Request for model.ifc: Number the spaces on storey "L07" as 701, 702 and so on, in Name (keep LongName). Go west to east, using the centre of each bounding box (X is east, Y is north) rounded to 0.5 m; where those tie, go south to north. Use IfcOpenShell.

First a look at what the model holds.

```python
import ifcopenshell
import ifcopenshell.util.element
import ifcopenshell.util.placement

model = ifcopenshell.open("model.ifc")
print(model.schema)
storey = next(s for s in model.by_type("IfcBuildingStorey") if s.Name == "L07")
spaces = [e for e in ifcopenshell.util.element.get_decomposition(storey) if e.is_a("IfcSpace")]
for e in sorted(spaces, key=lambda e: e.id()):
    origin = ifcopenshell.util.placement.get_local_placement(e.ObjectPlacement)[:3, 3]
    print(e.id(), e.Name, e.LongName, origin.round(2) + 0.0, sep=" | ")
```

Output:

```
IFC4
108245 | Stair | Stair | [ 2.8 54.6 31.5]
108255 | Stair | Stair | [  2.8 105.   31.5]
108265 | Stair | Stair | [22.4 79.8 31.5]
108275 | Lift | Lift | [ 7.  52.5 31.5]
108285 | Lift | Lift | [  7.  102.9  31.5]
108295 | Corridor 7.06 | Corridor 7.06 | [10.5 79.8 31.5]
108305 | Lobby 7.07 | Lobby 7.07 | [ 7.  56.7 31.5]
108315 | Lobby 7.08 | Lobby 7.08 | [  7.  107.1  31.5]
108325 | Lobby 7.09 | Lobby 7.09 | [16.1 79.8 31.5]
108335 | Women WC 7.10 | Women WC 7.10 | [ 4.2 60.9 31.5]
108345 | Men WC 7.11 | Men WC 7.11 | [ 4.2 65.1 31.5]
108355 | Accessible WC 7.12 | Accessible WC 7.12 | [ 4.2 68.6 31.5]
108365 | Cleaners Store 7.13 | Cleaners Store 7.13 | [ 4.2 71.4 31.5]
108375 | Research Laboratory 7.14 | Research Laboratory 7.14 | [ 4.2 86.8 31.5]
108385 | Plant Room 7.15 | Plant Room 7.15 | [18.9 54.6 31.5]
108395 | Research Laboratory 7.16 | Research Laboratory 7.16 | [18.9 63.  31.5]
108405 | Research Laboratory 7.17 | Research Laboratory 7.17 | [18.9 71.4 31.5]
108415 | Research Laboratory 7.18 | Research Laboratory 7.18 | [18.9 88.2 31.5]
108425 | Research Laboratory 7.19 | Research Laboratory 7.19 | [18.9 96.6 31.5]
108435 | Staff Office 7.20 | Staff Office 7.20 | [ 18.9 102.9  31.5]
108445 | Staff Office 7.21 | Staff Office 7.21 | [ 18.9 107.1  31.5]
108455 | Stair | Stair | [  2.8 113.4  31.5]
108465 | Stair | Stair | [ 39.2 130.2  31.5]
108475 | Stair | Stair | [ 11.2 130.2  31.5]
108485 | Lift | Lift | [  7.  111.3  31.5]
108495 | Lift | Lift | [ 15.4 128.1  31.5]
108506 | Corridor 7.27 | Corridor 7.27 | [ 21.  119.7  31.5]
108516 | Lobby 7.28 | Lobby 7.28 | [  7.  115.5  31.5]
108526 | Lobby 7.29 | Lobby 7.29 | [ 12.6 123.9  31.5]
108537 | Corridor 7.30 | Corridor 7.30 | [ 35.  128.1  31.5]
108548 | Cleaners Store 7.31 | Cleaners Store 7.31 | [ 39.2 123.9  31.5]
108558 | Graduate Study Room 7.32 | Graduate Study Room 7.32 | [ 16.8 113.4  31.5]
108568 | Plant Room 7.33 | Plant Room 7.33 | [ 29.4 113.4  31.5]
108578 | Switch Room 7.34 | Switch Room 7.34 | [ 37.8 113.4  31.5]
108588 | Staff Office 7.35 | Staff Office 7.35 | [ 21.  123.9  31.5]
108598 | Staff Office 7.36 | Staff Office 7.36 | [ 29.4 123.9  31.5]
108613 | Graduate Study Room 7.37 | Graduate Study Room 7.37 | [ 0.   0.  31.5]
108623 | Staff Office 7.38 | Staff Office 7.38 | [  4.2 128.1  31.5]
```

```python
import ifcopenshell
import ifcopenshell.geom
import ifcopenshell.util.element
import ifcopenshell.util.shape

model = ifcopenshell.open("model.ifc")
settings = ifcopenshell.geom.settings()
settings.set("use-world-coords", True)


def centre(element):
    shape = ifcopenshell.geom.create_shape(settings, element)
    return ifcopenshell.util.shape.get_bbox_centroid(shape.geometry)


storey = next(s for s in model.by_type("IfcBuildingStorey") if s.Name == "L07")
spaces = [e for e in ifcopenshell.util.element.get_decomposition(storey) if e.is_a("IfcSpace")]

# Insertion points can sit at a corner or the storey origin, so sort by the geometry (in metres).
centres = {e: centre(e) for e in spaces}
spaces.sort(key=lambda e: (round(centres[e][0] / 0.5), centres[e][1]))

for i, e in enumerate(spaces, start=1):
    number = f"7{i:02d}"
    e.Name = number
    print(e.id(), number)

model.write("model_rev.ifc")
```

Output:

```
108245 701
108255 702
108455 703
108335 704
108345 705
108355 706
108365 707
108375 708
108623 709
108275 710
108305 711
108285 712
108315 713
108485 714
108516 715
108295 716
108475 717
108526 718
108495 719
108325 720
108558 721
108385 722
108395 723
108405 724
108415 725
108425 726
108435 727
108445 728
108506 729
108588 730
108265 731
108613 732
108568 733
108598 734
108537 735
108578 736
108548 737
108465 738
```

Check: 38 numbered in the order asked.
